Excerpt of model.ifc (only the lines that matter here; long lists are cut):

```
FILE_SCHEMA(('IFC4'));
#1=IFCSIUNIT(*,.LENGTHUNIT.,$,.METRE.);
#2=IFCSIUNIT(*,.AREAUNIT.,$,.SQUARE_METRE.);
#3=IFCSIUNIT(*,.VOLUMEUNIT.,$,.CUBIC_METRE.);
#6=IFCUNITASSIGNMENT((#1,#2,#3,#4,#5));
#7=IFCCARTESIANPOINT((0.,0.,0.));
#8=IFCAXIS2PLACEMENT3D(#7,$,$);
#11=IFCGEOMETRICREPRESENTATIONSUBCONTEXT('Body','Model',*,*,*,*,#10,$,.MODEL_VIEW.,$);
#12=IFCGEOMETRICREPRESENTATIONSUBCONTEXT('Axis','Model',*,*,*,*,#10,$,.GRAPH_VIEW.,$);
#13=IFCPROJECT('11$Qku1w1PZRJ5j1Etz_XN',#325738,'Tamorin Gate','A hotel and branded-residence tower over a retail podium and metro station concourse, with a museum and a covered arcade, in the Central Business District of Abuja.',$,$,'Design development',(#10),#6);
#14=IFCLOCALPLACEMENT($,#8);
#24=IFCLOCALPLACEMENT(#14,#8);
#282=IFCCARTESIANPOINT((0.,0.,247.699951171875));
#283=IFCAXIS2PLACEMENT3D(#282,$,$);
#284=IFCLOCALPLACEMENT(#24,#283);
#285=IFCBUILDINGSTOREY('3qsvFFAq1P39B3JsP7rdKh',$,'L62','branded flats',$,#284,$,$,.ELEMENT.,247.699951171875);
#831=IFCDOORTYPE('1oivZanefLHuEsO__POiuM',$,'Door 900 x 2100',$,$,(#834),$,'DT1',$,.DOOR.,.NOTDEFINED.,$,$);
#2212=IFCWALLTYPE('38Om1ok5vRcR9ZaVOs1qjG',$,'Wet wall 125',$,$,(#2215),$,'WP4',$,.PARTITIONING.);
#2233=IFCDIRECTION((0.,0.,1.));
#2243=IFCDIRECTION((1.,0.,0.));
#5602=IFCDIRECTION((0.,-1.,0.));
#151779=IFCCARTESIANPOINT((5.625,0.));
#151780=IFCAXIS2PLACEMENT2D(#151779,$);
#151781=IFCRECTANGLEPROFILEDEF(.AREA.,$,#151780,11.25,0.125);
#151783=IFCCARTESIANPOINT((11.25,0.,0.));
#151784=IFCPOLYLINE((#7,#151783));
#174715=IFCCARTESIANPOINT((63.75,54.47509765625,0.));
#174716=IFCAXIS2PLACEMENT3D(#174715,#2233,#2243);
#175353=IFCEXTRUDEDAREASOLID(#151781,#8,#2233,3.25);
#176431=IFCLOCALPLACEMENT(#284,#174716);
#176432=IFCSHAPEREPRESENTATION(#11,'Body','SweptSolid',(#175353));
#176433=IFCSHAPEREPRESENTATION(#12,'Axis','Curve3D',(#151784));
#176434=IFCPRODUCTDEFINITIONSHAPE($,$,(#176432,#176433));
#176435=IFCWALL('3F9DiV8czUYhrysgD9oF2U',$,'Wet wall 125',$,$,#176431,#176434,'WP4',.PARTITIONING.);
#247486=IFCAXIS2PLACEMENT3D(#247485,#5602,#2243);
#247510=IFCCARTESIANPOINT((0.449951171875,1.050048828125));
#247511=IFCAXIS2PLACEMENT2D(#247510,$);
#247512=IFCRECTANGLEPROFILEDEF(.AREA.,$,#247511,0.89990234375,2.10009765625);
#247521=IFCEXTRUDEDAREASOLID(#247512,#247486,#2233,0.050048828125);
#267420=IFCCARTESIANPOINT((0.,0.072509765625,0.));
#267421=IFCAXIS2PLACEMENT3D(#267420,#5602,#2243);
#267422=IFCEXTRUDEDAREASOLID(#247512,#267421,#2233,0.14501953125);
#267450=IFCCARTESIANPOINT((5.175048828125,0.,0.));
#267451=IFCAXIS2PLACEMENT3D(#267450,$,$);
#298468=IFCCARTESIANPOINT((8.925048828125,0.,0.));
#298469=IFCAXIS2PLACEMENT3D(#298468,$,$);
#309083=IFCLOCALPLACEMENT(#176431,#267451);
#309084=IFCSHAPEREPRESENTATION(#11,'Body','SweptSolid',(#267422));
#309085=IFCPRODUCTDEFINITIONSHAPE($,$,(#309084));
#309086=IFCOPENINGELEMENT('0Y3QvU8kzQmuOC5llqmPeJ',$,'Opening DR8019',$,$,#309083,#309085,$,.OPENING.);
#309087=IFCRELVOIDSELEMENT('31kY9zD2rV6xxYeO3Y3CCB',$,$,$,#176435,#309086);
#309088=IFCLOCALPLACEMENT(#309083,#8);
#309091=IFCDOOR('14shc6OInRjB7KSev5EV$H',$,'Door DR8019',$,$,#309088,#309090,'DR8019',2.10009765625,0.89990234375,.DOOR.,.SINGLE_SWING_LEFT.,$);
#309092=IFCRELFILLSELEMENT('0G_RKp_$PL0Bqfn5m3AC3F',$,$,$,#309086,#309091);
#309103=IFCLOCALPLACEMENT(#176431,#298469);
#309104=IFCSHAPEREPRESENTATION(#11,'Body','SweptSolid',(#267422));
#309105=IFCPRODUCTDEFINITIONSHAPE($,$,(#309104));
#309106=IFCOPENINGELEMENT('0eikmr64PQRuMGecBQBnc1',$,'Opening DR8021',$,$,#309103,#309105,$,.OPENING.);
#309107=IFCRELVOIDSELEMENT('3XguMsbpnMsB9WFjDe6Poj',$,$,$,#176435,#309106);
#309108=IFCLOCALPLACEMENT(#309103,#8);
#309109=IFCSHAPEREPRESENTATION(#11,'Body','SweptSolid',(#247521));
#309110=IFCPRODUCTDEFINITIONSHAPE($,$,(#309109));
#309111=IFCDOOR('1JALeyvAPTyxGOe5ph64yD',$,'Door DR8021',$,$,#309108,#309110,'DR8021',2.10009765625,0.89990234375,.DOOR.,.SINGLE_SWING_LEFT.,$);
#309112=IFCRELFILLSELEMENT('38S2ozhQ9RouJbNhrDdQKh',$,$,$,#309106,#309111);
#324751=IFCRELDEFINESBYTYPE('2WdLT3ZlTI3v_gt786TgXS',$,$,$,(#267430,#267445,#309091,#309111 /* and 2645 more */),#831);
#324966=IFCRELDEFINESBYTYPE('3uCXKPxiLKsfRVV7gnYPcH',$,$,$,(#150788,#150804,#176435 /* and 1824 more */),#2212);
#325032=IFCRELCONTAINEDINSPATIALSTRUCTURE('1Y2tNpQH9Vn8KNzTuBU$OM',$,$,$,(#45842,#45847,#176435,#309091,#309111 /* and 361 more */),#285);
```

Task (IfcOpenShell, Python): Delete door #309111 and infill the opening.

```python
import ifcopenshell
import ifcopenshell.api.feature
import ifcopenshell.api.root
import ifcopenshell.geom
import ifcopenshell.util.shape

model = ifcopenshell.open("model.ifc")
settings = ifcopenshell.geom.settings()


def volume(element):
    """Net volume in cubic metres, openings subtracted."""
    shape = ifcopenshell.geom.create_shape(settings, element)
    return ifcopenshell.util.shape.get_volume(shape.geometry)


door = model.by_guid("1JALeyvAPTyxGOe5ph64yD")
opening = door.FillsVoids[0].RelatingOpeningElement
wall = opening.VoidsElements[0].RelatingBuildingElement
before = volume(wall)

ifcopenshell.api.root.remove_product(model, product=door)
ifcopenshell.api.feature.remove_feature(model, feature=opening)

after = volume(wall)

print(f"wall volume {before:.3f} -> {after:.3f} m3")

model.write("model_edited.ifc")
```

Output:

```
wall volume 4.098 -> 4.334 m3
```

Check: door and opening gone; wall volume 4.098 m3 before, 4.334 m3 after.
